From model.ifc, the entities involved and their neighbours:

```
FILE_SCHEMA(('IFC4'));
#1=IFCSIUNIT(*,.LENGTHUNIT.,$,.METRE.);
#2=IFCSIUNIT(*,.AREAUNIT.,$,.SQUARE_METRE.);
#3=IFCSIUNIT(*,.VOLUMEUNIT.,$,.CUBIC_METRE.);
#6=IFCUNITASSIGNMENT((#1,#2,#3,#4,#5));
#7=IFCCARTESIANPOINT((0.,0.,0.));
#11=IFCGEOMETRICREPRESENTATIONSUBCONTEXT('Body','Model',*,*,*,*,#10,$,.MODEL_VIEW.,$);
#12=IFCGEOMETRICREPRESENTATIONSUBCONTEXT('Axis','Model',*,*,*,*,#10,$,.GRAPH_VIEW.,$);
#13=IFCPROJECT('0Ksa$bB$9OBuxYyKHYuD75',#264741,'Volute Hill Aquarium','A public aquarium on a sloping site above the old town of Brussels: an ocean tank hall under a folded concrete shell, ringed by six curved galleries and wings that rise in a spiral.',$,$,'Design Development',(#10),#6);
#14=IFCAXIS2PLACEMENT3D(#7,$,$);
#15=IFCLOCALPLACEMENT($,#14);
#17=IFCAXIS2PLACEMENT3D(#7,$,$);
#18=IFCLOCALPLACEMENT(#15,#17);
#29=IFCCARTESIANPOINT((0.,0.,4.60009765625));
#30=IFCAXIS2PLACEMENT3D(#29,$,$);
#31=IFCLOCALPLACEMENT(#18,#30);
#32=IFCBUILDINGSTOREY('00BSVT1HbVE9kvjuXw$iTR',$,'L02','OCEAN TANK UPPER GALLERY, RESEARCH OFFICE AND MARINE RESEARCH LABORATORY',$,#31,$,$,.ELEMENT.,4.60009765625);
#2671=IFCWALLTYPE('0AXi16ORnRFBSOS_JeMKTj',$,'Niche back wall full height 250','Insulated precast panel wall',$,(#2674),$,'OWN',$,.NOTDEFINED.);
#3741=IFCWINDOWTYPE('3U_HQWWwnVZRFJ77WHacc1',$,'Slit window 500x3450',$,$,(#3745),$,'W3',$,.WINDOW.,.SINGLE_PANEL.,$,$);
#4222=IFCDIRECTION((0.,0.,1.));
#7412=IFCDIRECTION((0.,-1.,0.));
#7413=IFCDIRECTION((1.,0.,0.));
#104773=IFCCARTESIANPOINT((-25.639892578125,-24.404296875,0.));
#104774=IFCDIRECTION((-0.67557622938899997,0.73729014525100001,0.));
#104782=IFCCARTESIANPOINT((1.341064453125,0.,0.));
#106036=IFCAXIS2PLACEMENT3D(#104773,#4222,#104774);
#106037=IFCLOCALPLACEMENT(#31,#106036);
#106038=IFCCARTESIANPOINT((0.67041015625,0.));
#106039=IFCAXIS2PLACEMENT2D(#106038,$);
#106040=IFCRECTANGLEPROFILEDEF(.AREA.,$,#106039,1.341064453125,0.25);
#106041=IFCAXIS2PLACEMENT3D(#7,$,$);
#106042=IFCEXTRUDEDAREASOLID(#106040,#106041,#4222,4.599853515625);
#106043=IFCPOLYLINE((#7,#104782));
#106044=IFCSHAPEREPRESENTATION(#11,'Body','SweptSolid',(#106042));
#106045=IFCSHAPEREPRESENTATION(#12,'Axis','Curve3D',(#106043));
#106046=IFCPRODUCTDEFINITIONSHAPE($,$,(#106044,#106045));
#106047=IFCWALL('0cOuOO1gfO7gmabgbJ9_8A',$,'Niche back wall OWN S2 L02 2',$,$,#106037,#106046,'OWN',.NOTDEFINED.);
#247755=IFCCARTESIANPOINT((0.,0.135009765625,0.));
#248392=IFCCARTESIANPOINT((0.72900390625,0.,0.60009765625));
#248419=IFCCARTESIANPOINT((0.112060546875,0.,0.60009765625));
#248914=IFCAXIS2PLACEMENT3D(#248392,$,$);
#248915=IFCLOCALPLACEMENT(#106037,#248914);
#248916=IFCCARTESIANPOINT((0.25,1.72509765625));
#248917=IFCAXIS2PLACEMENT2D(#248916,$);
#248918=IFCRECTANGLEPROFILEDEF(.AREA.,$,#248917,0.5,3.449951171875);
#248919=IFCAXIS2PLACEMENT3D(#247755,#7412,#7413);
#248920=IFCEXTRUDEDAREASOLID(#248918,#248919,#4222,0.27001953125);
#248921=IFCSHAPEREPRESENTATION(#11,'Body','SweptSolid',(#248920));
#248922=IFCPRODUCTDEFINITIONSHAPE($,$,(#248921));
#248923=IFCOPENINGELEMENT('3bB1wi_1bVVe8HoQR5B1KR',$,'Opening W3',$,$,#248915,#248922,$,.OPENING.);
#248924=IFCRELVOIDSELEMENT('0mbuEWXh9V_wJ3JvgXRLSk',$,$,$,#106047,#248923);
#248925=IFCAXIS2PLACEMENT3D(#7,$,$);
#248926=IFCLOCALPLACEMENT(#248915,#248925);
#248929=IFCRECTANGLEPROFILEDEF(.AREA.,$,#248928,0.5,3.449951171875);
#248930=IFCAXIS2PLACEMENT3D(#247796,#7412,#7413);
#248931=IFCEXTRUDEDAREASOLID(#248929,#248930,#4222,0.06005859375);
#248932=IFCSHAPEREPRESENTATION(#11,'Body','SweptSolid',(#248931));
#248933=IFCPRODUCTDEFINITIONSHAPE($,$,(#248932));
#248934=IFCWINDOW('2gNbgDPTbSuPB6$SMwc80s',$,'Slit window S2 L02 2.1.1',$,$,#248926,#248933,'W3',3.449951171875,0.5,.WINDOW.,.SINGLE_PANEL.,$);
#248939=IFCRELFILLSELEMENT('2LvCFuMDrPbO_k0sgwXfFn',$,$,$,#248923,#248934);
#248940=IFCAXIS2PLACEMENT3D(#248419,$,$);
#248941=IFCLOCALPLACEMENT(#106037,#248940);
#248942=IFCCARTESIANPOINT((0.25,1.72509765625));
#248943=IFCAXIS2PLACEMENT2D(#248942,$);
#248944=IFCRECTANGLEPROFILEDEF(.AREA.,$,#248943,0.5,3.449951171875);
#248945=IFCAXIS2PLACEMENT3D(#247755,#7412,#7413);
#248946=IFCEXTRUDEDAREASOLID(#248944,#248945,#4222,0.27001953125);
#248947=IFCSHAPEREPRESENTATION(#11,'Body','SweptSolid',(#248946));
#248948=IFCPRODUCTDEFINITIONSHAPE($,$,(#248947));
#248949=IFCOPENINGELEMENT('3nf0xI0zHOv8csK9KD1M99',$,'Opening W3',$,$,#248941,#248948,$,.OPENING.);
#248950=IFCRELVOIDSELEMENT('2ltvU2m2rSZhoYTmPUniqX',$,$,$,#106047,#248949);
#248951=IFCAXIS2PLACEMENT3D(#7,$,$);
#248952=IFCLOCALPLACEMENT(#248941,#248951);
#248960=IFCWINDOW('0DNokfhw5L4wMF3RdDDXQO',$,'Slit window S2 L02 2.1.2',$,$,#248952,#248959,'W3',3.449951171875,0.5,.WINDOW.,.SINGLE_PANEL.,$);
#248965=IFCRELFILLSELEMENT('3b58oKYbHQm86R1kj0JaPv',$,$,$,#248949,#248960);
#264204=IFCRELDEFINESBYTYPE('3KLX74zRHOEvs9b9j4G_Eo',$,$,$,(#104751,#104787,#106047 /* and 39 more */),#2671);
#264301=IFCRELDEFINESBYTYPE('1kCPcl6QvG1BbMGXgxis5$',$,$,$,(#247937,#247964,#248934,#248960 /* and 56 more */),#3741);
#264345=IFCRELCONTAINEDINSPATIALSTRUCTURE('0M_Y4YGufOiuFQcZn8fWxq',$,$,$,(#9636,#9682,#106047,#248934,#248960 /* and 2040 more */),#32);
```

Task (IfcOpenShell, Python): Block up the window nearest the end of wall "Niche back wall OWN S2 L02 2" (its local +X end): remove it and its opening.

```python
import ifcopenshell
import ifcopenshell.api.feature
import ifcopenshell.api.root
import ifcopenshell.geom
import ifcopenshell.util.shape

model = ifcopenshell.open("model.ifc")
settings = ifcopenshell.geom.settings()


def volume(element):
    """Net volume in cubic metres, openings subtracted."""
    shape = ifcopenshell.geom.create_shape(settings, element)
    return ifcopenshell.util.shape.get_volume(shape.geometry)


window = model.by_guid("2gNbgDPTbSuPB6$SMwc80s")
opening = window.FillsVoids[0].RelatingOpeningElement
wall = opening.VoidsElements[0].RelatingBuildingElement
before = volume(wall)

ifcopenshell.api.root.remove_product(model, product=window)
ifcopenshell.api.feature.remove_feature(model, feature=opening)

after = volume(wall)

print(f"wall volume {before:.3f} -> {after:.3f} m3")

model.write("model_rev.ifc")
```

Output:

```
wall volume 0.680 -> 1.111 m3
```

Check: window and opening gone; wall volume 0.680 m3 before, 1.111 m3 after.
